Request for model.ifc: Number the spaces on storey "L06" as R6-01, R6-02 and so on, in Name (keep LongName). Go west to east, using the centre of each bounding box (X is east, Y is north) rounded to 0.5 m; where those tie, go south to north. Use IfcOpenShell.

First a look at what the model holds.

```python
import ifcopenshell
import ifcopenshell.util.element
import ifcopenshell.util.placement

model = ifcopenshell.open("model.ifc")
print(model.schema)
storey = next(s for s in model.by_type("IfcBuildingStorey") if s.Name == "L06")
spaces = [e for e in ifcopenshell.util.element.get_decomposition(storey) if e.is_a("IfcSpace")]
for e in sorted(spaces, key=lambda e: e.id()):
    origin = ifcopenshell.util.placement.get_local_placement(e.ObjectPlacement)[:3, 3]
    print(e.id(), e.Name, e.LongName, origin.round(2) + 0.0, sep=" | ")
```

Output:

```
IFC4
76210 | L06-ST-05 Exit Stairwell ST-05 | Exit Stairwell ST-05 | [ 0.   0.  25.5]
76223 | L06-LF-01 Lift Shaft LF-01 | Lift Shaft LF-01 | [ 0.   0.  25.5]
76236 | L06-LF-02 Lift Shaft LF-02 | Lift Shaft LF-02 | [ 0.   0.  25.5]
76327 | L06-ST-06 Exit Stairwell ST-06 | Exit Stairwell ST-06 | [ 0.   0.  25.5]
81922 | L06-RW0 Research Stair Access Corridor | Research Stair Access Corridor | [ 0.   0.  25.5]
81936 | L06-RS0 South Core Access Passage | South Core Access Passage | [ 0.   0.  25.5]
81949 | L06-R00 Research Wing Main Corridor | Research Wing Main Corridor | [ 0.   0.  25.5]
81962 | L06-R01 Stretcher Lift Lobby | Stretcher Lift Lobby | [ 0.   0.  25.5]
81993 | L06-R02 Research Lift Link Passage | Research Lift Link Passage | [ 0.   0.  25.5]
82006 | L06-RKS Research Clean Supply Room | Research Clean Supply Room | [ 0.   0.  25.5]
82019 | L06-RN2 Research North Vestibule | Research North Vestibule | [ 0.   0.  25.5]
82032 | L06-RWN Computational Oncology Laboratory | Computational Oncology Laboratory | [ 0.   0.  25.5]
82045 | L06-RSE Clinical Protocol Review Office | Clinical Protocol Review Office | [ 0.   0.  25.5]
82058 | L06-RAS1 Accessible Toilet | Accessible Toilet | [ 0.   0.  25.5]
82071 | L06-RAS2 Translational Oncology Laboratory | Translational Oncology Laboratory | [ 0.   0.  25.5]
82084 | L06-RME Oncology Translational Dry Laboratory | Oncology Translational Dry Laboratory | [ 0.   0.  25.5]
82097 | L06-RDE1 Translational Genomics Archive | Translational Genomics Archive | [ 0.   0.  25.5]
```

```python
import ifcopenshell
import ifcopenshell.geom
import ifcopenshell.util.element
import ifcopenshell.util.shape

model = ifcopenshell.open("model.ifc")
settings = ifcopenshell.geom.settings()
settings.set("use-world-coords", True)


def centre(element):
    shape = ifcopenshell.geom.create_shape(settings, element)
    return ifcopenshell.util.shape.get_bbox_centroid(shape.geometry)


storey = next(s for s in model.by_type("IfcBuildingStorey") if s.Name == "L06")
spaces = [e for e in ifcopenshell.util.element.get_decomposition(storey) if e.is_a("IfcSpace")]

# Insertion points can sit at a corner or the storey origin, so sort by the geometry (in metres).
centres = {e: centre(e) for e in spaces}
spaces.sort(key=lambda e: (round(centres[e][0] / 0.5), centres[e][1]))

for i, e in enumerate(spaces, start=1):
    number = f"R6-{i:02d}"
    e.Name = number
    print(e.id(), number)

model.write("model_edited.ifc")
```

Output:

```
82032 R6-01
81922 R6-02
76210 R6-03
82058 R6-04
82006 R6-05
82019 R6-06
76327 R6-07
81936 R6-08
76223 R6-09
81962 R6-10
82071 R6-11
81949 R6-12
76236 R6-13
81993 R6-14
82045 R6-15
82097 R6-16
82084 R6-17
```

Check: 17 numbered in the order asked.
